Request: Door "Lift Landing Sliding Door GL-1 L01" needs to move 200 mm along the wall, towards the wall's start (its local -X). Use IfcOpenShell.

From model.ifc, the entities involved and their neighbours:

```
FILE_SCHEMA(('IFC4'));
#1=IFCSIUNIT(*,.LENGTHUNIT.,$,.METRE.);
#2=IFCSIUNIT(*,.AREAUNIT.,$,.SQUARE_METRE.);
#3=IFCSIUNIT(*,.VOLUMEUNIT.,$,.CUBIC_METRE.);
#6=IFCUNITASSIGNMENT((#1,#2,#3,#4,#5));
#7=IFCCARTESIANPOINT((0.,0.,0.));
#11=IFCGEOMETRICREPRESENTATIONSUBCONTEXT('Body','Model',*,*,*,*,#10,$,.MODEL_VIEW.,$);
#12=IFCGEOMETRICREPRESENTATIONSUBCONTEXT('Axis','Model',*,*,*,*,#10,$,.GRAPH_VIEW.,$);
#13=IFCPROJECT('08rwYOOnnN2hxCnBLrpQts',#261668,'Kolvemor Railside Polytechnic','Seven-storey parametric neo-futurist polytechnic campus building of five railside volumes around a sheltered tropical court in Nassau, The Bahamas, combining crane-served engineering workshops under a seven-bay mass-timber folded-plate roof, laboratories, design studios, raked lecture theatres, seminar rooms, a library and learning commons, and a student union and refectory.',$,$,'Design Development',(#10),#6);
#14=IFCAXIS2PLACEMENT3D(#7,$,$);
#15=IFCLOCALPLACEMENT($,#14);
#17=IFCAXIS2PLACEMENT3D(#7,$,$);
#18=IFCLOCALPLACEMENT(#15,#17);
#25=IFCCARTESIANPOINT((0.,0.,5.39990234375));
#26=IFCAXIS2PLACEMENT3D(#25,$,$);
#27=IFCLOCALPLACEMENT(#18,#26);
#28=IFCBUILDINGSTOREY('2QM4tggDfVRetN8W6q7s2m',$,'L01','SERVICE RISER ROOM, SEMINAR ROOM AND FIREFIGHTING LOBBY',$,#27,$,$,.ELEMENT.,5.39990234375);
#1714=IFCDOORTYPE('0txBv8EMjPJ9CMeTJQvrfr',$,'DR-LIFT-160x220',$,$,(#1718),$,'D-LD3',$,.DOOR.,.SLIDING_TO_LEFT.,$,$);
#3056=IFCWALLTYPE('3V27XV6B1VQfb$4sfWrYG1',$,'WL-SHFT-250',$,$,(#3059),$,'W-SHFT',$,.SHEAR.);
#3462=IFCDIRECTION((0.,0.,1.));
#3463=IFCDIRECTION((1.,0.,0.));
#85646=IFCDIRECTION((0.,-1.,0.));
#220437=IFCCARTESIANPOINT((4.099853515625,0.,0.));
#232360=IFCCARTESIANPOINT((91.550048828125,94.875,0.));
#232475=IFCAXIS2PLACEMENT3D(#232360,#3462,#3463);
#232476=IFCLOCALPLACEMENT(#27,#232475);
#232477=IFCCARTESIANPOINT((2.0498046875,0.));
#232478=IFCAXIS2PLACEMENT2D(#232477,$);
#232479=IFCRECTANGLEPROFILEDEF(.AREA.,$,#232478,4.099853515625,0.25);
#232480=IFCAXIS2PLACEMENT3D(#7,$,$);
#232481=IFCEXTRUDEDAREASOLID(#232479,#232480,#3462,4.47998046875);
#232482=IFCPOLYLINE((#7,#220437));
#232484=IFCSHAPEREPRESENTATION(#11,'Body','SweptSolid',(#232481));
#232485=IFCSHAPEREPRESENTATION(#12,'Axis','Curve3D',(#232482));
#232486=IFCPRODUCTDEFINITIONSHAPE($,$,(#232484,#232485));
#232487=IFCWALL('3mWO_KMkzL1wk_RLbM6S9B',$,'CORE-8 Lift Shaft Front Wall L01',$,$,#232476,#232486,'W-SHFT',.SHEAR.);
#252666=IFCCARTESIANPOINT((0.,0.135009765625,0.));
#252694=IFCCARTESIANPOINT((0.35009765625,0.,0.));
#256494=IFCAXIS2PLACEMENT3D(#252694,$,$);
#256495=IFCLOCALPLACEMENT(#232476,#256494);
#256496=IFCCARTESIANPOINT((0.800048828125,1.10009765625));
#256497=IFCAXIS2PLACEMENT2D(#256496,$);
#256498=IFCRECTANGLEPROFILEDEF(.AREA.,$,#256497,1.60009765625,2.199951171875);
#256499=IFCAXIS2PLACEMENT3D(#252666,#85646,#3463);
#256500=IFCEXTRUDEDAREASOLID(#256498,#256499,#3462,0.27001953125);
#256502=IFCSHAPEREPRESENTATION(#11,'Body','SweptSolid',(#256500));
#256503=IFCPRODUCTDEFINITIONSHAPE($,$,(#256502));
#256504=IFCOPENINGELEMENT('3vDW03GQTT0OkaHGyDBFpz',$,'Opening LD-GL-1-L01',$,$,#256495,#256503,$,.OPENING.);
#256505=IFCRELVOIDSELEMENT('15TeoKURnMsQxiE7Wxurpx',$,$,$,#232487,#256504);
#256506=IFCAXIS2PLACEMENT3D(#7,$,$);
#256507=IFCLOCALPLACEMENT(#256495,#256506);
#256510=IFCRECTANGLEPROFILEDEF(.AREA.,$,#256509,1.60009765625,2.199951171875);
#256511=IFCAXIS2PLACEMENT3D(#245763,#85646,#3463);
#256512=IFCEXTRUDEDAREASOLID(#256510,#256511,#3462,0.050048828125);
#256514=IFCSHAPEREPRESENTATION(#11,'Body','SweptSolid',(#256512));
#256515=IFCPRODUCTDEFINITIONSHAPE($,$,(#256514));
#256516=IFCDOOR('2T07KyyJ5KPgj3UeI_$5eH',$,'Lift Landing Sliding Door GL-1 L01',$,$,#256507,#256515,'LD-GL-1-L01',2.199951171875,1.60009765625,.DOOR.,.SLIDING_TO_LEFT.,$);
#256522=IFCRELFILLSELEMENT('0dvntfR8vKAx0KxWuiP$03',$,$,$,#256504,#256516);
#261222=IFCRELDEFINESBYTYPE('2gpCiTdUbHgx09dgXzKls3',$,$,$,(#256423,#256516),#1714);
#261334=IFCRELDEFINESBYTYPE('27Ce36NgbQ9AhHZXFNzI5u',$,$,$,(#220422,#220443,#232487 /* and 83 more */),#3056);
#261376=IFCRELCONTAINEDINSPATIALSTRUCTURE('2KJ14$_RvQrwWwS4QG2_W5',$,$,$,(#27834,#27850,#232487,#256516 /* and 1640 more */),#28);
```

```python
import ifcopenshell
import ifcopenshell.api.geometry
import ifcopenshell.util.placement

model = ifcopenshell.open("model.ifc")

door = model.by_guid("2T07KyyJ5KPgj3UeI_$5eH")
opening = door.FillsVoids[0].RelatingOpeningElement
wall = opening.VoidsElements[0].RelatingBuildingElement

wall_matrix = ifcopenshell.util.placement.get_local_placement(wall.ObjectPlacement)
shift = wall_matrix[:3, 0] * -0.2
before = ifcopenshell.util.placement.get_local_placement(door.ObjectPlacement)[:3, 3].copy()

# The door is placed relative to its opening, so it follows when the opening moves.
matrix = ifcopenshell.util.placement.get_local_placement(opening.ObjectPlacement)
matrix[:3, 3] += shift
ifcopenshell.api.geometry.edit_object_placement(
    model, product=opening, matrix=matrix, is_si=False, should_transform_children=True
)

after = ifcopenshell.util.placement.get_local_placement(door.ObjectPlacement)[:3, 3]
print("door moved by", (after - before).round(3) + 0.0)

model.write("model_updated.ifc")
```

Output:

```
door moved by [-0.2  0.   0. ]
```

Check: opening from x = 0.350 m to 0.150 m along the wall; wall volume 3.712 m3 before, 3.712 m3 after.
